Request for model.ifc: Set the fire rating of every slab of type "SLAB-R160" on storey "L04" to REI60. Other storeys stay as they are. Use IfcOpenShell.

First a look at what the model holds.

```python
import ifcopenshell
import ifcopenshell.util.element

model = ifcopenshell.open("model.ifc")
print(model.schema)
storey = next(s for s in model.by_type("IfcBuildingStorey") if s.Name == "L04")
slabs = [e for e in ifcopenshell.util.element.get_decomposition(storey) if e.is_a("IfcSlab")]
seen = {}
for e in slabs:
    element_type = ifcopenshell.util.element.get_type(e)
    key = (element_type.Name if element_type != e and element_type else None, ifcopenshell.util.element.get_pset(e, "Pset_SlabCommon", "FireRating"))
    seen[key] = seen.get(key, 0) + 1
for (name, value), count in sorted(seen.items(), key=str):
    print(count, "x", name, "|", value)
```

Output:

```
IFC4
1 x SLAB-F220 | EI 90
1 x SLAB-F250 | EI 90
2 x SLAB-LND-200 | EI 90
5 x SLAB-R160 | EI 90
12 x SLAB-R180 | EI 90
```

```python
import ifcopenshell
import ifcopenshell.api.pset
import ifcopenshell.util.element

model = ifcopenshell.open("model.ifc")

storey = next(s for s in model.by_type("IfcBuildingStorey") if s.Name == "L04")
slabs = [e for e in ifcopenshell.util.element.get_decomposition(storey) if e.is_a("IfcSlab")]

count = 0
for e in slabs:
    element_type = ifcopenshell.util.element.get_type(e)
    if element_type in (None, e) or element_type.Name != "SLAB-R160":
        continue
    # add_pset returns the element's existing set when there is one.
    pset = ifcopenshell.api.pset.add_pset(model, product=e, name="Pset_SlabCommon")
    ifcopenshell.api.pset.edit_pset(model, pset=pset, properties={"FireRating": "REI60"})
    count += 1

print(count, "slabs updated")

model.write("model-out.ifc")
```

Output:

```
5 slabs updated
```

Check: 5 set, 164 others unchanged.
